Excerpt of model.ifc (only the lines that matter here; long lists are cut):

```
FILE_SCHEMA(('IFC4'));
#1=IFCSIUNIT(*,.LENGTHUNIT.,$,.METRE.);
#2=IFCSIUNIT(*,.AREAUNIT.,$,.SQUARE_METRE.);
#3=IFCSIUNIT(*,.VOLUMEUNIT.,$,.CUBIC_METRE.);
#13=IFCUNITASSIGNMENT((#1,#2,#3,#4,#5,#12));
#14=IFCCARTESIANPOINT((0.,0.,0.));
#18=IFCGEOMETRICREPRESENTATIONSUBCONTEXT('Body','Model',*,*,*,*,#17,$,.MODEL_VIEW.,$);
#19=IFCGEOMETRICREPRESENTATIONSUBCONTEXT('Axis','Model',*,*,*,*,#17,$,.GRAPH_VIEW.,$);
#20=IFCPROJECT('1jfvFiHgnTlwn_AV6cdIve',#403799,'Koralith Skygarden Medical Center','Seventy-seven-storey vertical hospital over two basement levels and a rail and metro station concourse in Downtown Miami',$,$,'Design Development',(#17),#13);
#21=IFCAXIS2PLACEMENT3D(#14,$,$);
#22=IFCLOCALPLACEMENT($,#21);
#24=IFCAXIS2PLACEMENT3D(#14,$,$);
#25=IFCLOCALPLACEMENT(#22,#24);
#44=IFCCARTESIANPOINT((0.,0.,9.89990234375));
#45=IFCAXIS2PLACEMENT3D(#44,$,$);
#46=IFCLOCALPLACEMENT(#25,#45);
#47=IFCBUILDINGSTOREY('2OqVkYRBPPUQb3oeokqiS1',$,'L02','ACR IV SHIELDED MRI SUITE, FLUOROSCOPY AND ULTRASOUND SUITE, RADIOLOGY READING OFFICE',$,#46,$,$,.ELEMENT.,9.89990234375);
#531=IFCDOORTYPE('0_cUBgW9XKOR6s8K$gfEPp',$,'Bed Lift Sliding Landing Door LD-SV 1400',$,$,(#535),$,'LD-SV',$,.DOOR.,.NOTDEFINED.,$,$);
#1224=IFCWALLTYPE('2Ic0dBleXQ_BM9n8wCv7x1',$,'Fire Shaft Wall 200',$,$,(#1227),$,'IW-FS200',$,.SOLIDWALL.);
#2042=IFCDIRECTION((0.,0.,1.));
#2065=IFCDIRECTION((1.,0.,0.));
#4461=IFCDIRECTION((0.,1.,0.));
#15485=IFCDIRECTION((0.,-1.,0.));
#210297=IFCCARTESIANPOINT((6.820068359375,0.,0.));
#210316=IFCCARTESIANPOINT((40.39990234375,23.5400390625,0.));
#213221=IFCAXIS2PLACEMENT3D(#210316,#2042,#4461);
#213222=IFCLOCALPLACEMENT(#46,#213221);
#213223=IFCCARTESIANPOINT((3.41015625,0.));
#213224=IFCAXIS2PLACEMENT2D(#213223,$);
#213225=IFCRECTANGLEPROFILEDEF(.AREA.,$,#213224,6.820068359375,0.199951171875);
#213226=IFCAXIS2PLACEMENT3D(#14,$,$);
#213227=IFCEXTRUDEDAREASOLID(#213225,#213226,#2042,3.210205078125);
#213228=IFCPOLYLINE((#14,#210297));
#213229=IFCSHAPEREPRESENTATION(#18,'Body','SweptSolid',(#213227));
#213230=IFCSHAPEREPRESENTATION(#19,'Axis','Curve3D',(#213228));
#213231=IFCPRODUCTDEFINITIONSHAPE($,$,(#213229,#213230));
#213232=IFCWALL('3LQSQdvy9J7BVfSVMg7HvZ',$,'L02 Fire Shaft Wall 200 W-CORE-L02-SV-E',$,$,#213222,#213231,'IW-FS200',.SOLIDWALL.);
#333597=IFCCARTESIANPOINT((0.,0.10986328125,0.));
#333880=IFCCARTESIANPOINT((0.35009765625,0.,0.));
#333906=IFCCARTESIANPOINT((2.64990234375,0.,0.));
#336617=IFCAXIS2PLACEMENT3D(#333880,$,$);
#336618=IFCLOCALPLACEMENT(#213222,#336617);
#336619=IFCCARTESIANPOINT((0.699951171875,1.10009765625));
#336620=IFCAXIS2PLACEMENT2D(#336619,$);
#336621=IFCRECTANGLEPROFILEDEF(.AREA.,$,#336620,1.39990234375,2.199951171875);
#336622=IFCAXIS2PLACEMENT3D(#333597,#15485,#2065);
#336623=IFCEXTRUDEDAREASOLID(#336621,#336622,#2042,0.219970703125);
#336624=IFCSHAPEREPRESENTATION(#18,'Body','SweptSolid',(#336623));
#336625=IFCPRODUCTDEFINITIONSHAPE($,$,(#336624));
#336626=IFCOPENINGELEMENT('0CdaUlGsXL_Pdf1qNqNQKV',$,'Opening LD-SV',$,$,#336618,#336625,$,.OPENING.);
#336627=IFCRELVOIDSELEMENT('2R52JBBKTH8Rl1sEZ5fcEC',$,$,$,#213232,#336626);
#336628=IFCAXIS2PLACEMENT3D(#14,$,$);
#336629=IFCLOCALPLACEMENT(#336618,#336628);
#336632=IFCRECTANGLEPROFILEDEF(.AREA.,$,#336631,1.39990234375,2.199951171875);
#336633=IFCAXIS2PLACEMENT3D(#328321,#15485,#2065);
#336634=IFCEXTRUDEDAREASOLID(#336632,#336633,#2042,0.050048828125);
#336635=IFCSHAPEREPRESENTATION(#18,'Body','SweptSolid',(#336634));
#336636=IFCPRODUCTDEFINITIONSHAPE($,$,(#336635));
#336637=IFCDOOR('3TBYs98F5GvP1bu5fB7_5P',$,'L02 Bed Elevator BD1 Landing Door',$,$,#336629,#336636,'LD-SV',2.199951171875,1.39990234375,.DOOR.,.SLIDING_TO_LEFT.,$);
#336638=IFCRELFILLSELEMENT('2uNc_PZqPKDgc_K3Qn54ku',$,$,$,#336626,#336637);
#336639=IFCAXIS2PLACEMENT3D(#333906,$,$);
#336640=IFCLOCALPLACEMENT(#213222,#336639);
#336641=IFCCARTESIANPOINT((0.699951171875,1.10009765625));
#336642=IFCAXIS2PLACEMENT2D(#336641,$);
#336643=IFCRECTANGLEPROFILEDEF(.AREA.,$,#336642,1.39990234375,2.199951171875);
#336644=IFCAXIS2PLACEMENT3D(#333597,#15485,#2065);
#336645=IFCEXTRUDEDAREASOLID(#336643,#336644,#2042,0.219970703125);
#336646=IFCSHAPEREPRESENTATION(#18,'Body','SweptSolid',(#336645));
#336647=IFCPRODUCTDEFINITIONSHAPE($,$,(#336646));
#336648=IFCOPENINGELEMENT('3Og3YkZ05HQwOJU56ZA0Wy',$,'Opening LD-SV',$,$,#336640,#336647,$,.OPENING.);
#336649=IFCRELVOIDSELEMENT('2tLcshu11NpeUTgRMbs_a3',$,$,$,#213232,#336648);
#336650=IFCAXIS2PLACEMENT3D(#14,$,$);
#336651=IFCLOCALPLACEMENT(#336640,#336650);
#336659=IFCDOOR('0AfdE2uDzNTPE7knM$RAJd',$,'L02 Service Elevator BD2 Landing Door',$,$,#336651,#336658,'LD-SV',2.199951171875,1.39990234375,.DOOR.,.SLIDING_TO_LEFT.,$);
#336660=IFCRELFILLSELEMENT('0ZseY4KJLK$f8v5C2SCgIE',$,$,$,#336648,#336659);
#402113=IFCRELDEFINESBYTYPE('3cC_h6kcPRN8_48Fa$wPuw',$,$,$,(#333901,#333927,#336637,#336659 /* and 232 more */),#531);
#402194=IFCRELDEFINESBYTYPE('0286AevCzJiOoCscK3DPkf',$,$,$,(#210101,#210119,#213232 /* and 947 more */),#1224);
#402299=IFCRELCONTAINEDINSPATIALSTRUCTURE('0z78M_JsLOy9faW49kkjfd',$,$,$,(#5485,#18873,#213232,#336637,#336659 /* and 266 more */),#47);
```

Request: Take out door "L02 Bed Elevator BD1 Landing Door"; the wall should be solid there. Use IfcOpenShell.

```python
import ifcopenshell
import ifcopenshell.api.feature
import ifcopenshell.api.root
import ifcopenshell.geom
import ifcopenshell.util.shape

model = ifcopenshell.open("model.ifc")
settings = ifcopenshell.geom.settings()


def volume(element):
    """Net volume in cubic metres, openings subtracted."""
    shape = ifcopenshell.geom.create_shape(settings, element)
    return ifcopenshell.util.shape.get_volume(shape.geometry)


door = model.by_guid("3TBYs98F5GvP1bu5fB7_5P")
opening = door.FillsVoids[0].RelatingOpeningElement
wall = opening.VoidsElements[0].RelatingBuildingElement
before = volume(wall)

ifcopenshell.api.root.remove_product(model, product=door)
ifcopenshell.api.feature.remove_feature(model, feature=opening)

after = volume(wall)

print(f"wall volume {before:.3f} -> {after:.3f} m3")

model.write("model_updated.ifc")
```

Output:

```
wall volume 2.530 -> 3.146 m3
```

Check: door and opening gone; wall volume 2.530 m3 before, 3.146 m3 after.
